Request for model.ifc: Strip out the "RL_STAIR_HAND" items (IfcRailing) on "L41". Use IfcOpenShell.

First a look at what the model holds.

```python
import ifcopenshell
import ifcopenshell.util.element

model = ifcopenshell.open("model.ifc")
print(model.schema)
storey = next(s for s in model.by_type("IfcBuildingStorey") if s.Name == "L41")
railings = [e for e in ifcopenshell.util.element.get_decomposition(storey) if e.is_a("IfcRailing")]
seen = {}
for e in railings:
    element_type = ifcopenshell.util.element.get_type(e)
    name = element_type.Name if element_type not in (None, e) else None
    seen[name] = seen.get(name, 0) + 1
for name, count in sorted(seen.items(), key=str):
    print(count, "x", name)
```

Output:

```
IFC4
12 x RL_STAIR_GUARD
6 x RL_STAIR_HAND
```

```python
import ifcopenshell
import ifcopenshell.api.root
import ifcopenshell.util.element

model = ifcopenshell.open("model.ifc")

storey = next(s for s in model.by_type("IfcBuildingStorey") if s.Name == "L41")
railings = [e for e in ifcopenshell.util.element.get_decomposition(storey) if e.is_a("IfcRailing")]
targets = [e for e in railings if (t := ifcopenshell.util.element.get_type(e)) not in (None, e) and t.Name == "RL_STAIR_HAND"]

for e in targets:
    ifcopenshell.api.root.remove_product(model, product=e)
print(len(targets), "removed")

model.write("model_v2.ifc")
```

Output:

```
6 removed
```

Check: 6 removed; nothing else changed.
